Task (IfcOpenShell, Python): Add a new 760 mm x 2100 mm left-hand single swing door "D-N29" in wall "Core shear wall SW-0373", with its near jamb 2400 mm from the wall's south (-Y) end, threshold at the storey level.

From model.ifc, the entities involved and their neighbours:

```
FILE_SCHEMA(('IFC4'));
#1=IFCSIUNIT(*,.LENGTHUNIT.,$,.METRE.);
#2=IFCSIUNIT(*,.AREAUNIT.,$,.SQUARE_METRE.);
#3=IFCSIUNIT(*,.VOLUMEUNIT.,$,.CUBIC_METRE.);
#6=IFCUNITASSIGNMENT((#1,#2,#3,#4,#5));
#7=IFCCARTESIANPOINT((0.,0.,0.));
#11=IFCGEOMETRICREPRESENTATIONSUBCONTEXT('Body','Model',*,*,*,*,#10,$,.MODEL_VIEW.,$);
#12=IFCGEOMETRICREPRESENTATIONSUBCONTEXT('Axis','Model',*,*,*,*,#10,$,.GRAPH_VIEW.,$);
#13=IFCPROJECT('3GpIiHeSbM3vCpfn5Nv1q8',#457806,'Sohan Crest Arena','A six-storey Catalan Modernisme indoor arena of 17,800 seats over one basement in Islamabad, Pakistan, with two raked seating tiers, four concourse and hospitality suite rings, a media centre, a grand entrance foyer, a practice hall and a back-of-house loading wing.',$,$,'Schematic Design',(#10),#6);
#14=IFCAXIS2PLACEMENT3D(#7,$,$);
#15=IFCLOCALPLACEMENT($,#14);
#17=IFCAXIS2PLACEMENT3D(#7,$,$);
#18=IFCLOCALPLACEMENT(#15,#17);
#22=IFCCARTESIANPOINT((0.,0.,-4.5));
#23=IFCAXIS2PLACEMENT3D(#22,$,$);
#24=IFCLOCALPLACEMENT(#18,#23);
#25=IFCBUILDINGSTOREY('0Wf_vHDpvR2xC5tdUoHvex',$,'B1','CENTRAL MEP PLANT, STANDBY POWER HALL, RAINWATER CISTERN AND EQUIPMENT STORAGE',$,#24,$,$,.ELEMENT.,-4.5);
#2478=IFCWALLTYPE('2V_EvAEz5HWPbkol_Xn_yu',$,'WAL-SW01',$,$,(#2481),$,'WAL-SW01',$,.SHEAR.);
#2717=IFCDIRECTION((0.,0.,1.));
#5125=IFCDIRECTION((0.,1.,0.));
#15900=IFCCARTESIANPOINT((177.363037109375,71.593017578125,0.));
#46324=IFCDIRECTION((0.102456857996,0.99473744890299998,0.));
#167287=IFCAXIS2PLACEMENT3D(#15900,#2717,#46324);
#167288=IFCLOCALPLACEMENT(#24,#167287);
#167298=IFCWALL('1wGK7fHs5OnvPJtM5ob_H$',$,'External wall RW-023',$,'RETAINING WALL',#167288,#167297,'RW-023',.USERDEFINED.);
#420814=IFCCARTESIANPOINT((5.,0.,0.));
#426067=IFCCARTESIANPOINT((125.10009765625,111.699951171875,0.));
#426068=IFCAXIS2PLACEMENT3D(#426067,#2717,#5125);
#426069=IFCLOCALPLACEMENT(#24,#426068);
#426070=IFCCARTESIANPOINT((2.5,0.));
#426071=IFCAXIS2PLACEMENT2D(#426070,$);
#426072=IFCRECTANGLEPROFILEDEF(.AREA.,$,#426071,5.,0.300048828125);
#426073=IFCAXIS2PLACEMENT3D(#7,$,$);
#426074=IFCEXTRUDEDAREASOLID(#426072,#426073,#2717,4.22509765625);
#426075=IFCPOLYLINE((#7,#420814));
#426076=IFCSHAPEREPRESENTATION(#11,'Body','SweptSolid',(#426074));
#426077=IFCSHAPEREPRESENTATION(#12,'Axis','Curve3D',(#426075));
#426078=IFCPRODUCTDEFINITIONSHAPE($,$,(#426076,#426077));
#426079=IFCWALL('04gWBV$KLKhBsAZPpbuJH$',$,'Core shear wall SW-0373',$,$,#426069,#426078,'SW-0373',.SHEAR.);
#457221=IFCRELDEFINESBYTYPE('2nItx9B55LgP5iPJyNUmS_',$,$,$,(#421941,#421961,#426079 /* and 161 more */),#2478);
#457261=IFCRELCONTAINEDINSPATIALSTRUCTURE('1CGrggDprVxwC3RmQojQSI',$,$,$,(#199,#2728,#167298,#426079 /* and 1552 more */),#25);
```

```python
import numpy as np
import ifcopenshell
import ifcopenshell.api.feature
import ifcopenshell.api.geometry
import ifcopenshell.api.root
import ifcopenshell.api.spatial
import ifcopenshell.geom
import ifcopenshell.util.element
import ifcopenshell.util.placement
import ifcopenshell.util.representation
import ifcopenshell.util.shape
import ifcopenshell.util.unit

model = ifcopenshell.open("model.ifc")
unit_scale = ifcopenshell.util.unit.calculate_unit_scale(model)
settings = ifcopenshell.geom.settings()


def volume(element):
    """Net volume in cubic metres, openings subtracted."""
    shape = ifcopenshell.geom.create_shape(settings, element)
    return ifcopenshell.util.shape.get_volume(shape.geometry)


wall = model.by_guid("04gWBV$KLKhBsAZPpbuJH$")
storey = ifcopenshell.util.element.get_container(wall, ifc_class="IfcBuildingStorey")
context = ifcopenshell.util.representation.get_context(model, "Model", "Body", "MODEL_VIEW")
before = volume(wall)

width, height, from_end, sill = 0.76, 2.1, 2.4, 0.0  # metres

# The wall runs along its own X axis, and the end named is its -X end.
wall_shape = ifcopenshell.geom.create_shape(settings, wall)
x, y, z = ifcopenshell.util.shape.get_vertices(wall_shape.geometry).T
start = x.min() + from_end
face, thickness = float(y.min()), float(y.max() - y.min())
wall_matrix = ifcopenshell.util.placement.get_local_placement(wall.ObjectPlacement)
level = ifcopenshell.util.placement.get_local_placement(storey.ObjectPlacement)[2, 3]


def in_wall(x, y):
    """Placement at x, y metres in the wall's axes, at sill height."""
    matrix = wall_matrix.copy()
    matrix[:, 3] = wall_matrix @ np.array([x / unit_scale, y / unit_scale, 0.0, 1.0])
    matrix[2, 3] = level + sill / unit_scale
    return matrix


# Opening: a box that overshoots both wall faces by 50 mm.
opening = ifcopenshell.api.root.create_entity(model, ifc_class="IfcOpeningElement", predefined_type="OPENING")
box = ifcopenshell.api.geometry.add_wall_representation(
    model, context=context, length=width, height=height, thickness=thickness + 0.1
)
ifcopenshell.api.geometry.assign_representation(model, product=opening, representation=box)
ifcopenshell.api.geometry.edit_object_placement(model, product=opening, matrix=in_wall(start, face - 0.05), is_si=False)
ifcopenshell.api.feature.add_feature(model, feature=opening, element=wall)

door = ifcopenshell.api.root.create_entity(model, ifc_class="IfcDoor", name="D-N29", predefined_type="DOOR")
door.OverallWidth, door.OverallHeight = width / unit_scale, height / unit_scale
door.OperationType = "SINGLE_SWING_LEFT"
body = ifcopenshell.api.geometry.add_door_representation(
    model,
    context=context,
    overall_width=door.OverallWidth,
    overall_height=door.OverallHeight,
    operation_type="SINGLE_SWING_LEFT",
    lining_properties={"LiningDepth": thickness / unit_scale, "ThresholdDepth": thickness / unit_scale},
)
ifcopenshell.api.geometry.assign_representation(model, product=door, representation=body)
ifcopenshell.api.spatial.assign_container(model, products=[door], relating_structure=storey)
ifcopenshell.api.feature.add_filling(model, opening=opening, element=door)

# The lining spans the wall, so the door starts at the wall face.
ifcopenshell.api.geometry.edit_object_placement(model, product=door, matrix=in_wall(start, face), is_si=False)

after = volume(wall)

print(f"wall volume {before:.3f} -> {after:.3f} m3")

model.write("model_rev.ifc")
```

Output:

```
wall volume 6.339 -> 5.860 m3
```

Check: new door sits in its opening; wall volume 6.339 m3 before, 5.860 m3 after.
